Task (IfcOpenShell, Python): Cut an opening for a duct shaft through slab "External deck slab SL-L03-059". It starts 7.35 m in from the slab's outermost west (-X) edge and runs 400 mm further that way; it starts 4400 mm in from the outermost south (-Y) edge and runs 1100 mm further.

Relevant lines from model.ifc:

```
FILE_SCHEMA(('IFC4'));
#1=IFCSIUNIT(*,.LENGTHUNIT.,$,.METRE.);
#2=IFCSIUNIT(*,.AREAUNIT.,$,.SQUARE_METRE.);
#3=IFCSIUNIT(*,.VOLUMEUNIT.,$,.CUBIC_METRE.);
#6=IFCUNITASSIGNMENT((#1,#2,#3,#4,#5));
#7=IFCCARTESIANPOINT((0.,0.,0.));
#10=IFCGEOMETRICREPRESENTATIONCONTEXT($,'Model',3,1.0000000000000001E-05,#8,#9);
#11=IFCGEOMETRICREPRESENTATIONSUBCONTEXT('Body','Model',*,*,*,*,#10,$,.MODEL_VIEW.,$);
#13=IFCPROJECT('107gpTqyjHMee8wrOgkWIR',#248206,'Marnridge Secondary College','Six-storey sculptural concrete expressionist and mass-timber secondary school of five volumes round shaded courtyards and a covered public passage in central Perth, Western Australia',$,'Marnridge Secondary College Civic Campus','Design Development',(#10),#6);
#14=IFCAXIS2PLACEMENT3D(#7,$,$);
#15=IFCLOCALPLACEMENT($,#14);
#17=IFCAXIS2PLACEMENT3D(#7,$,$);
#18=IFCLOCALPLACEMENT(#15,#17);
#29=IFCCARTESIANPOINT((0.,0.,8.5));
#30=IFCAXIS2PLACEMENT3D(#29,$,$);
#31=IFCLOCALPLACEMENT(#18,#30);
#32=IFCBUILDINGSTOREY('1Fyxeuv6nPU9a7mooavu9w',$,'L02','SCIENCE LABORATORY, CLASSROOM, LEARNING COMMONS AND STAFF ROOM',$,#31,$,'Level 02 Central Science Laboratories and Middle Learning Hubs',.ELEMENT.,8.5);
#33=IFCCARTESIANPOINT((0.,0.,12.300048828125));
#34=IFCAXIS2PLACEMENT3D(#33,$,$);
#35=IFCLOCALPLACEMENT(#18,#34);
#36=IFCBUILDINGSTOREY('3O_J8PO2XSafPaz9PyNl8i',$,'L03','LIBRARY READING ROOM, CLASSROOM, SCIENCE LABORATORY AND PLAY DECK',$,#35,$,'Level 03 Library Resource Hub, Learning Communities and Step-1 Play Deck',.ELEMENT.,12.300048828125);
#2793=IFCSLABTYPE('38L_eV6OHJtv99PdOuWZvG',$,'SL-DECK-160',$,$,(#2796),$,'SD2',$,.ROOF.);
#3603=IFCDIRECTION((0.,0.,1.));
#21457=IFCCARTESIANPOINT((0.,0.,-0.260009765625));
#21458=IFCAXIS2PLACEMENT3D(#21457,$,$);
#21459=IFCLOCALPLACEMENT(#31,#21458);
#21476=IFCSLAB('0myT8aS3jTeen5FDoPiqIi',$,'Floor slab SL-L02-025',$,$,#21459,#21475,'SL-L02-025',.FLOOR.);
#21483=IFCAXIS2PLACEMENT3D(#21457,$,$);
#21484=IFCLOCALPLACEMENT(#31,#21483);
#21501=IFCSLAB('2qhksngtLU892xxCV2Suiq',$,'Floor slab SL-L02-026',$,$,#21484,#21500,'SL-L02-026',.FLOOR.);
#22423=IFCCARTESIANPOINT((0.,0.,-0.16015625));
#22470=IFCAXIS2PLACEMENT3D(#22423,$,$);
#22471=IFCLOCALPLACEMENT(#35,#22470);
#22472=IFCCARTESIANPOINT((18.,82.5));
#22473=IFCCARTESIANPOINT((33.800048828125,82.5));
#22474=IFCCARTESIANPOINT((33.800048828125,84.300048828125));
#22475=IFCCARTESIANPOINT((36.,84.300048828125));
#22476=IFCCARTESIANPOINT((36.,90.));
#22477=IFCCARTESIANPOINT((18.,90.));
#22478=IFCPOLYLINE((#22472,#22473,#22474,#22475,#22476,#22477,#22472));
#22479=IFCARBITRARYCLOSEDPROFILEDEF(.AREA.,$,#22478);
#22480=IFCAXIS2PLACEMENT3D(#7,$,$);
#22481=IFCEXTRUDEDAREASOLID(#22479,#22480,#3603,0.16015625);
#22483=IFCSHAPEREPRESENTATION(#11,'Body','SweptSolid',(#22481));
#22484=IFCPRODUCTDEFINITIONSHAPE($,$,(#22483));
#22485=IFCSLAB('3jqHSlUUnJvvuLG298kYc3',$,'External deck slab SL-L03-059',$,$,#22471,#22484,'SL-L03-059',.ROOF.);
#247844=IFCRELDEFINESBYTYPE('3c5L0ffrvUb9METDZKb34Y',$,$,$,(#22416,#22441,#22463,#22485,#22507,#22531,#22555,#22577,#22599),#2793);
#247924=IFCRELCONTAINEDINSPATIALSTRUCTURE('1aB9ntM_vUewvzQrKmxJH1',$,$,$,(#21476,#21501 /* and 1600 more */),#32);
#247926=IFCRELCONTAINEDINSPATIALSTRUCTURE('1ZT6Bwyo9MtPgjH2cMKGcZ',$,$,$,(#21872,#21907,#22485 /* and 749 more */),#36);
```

```python
import numpy as np
import ifcopenshell
import ifcopenshell.api.feature
import ifcopenshell.api.geometry
import ifcopenshell.api.root
import ifcopenshell.geom
import ifcopenshell.util.placement
import ifcopenshell.util.representation
import ifcopenshell.util.shape
import ifcopenshell.util.unit

model = ifcopenshell.open("model.ifc")
unit_scale = ifcopenshell.util.unit.calculate_unit_scale(model)
settings = ifcopenshell.geom.settings()


def volume(element):
    """Net volume in cubic metres, openings subtracted."""
    shape = ifcopenshell.geom.create_shape(settings, element)
    return ifcopenshell.util.shape.get_volume(shape.geometry)


slab = model.by_guid("3jqHSlUUnJvvuLG298kYc3")
before = volume(slab)

# Extent in the slab's own axes, in metres. The edges named are its -X and -Y sides.
slab_shape = ifcopenshell.geom.create_shape(settings, slab)
vertices = ifcopenshell.util.shape.get_vertices(slab_shape.geometry)
x_min, y_min, bottom = vertices.min(axis=0)
top = vertices[:, 2].max()

opening = ifcopenshell.api.root.create_entity(model, ifc_class="IfcOpeningElement", name="Duct shaft opening", predefined_type="OPENING")
context = ifcopenshell.util.representation.get_context(model, "Model", "Body", "MODEL_VIEW")
width, depth = 0.4, 1.1
outline = [(0.0, 0.0), (width, 0.0), (width, depth), (0.0, depth), (0.0, 0.0)]
# Overshoot both faces by 50 mm so the cut is clean.
shape = ifcopenshell.api.geometry.add_slab_representation(
    model, context=context, depth=top - bottom + 0.1, polyline=outline
)
ifcopenshell.api.geometry.assign_representation(model, product=opening, representation=shape)

matrix = ifcopenshell.util.placement.get_local_placement(slab.ObjectPlacement)
matrix[:, 3] = matrix @ np.append(np.array([x_min + 7.35, y_min + 4.4, bottom - 0.05]) / unit_scale, 1.0)
ifcopenshell.api.geometry.edit_object_placement(model, product=opening, matrix=matrix, is_si=False)
ifcopenshell.api.feature.add_feature(model, feature=opening, element=slab)

after = volume(slab)

print(f"slab volume {before:.3f} -> {after:.3f} m3")

model.write("model-out.ifc")
```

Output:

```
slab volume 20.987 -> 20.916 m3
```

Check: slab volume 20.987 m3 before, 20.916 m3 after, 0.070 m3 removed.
